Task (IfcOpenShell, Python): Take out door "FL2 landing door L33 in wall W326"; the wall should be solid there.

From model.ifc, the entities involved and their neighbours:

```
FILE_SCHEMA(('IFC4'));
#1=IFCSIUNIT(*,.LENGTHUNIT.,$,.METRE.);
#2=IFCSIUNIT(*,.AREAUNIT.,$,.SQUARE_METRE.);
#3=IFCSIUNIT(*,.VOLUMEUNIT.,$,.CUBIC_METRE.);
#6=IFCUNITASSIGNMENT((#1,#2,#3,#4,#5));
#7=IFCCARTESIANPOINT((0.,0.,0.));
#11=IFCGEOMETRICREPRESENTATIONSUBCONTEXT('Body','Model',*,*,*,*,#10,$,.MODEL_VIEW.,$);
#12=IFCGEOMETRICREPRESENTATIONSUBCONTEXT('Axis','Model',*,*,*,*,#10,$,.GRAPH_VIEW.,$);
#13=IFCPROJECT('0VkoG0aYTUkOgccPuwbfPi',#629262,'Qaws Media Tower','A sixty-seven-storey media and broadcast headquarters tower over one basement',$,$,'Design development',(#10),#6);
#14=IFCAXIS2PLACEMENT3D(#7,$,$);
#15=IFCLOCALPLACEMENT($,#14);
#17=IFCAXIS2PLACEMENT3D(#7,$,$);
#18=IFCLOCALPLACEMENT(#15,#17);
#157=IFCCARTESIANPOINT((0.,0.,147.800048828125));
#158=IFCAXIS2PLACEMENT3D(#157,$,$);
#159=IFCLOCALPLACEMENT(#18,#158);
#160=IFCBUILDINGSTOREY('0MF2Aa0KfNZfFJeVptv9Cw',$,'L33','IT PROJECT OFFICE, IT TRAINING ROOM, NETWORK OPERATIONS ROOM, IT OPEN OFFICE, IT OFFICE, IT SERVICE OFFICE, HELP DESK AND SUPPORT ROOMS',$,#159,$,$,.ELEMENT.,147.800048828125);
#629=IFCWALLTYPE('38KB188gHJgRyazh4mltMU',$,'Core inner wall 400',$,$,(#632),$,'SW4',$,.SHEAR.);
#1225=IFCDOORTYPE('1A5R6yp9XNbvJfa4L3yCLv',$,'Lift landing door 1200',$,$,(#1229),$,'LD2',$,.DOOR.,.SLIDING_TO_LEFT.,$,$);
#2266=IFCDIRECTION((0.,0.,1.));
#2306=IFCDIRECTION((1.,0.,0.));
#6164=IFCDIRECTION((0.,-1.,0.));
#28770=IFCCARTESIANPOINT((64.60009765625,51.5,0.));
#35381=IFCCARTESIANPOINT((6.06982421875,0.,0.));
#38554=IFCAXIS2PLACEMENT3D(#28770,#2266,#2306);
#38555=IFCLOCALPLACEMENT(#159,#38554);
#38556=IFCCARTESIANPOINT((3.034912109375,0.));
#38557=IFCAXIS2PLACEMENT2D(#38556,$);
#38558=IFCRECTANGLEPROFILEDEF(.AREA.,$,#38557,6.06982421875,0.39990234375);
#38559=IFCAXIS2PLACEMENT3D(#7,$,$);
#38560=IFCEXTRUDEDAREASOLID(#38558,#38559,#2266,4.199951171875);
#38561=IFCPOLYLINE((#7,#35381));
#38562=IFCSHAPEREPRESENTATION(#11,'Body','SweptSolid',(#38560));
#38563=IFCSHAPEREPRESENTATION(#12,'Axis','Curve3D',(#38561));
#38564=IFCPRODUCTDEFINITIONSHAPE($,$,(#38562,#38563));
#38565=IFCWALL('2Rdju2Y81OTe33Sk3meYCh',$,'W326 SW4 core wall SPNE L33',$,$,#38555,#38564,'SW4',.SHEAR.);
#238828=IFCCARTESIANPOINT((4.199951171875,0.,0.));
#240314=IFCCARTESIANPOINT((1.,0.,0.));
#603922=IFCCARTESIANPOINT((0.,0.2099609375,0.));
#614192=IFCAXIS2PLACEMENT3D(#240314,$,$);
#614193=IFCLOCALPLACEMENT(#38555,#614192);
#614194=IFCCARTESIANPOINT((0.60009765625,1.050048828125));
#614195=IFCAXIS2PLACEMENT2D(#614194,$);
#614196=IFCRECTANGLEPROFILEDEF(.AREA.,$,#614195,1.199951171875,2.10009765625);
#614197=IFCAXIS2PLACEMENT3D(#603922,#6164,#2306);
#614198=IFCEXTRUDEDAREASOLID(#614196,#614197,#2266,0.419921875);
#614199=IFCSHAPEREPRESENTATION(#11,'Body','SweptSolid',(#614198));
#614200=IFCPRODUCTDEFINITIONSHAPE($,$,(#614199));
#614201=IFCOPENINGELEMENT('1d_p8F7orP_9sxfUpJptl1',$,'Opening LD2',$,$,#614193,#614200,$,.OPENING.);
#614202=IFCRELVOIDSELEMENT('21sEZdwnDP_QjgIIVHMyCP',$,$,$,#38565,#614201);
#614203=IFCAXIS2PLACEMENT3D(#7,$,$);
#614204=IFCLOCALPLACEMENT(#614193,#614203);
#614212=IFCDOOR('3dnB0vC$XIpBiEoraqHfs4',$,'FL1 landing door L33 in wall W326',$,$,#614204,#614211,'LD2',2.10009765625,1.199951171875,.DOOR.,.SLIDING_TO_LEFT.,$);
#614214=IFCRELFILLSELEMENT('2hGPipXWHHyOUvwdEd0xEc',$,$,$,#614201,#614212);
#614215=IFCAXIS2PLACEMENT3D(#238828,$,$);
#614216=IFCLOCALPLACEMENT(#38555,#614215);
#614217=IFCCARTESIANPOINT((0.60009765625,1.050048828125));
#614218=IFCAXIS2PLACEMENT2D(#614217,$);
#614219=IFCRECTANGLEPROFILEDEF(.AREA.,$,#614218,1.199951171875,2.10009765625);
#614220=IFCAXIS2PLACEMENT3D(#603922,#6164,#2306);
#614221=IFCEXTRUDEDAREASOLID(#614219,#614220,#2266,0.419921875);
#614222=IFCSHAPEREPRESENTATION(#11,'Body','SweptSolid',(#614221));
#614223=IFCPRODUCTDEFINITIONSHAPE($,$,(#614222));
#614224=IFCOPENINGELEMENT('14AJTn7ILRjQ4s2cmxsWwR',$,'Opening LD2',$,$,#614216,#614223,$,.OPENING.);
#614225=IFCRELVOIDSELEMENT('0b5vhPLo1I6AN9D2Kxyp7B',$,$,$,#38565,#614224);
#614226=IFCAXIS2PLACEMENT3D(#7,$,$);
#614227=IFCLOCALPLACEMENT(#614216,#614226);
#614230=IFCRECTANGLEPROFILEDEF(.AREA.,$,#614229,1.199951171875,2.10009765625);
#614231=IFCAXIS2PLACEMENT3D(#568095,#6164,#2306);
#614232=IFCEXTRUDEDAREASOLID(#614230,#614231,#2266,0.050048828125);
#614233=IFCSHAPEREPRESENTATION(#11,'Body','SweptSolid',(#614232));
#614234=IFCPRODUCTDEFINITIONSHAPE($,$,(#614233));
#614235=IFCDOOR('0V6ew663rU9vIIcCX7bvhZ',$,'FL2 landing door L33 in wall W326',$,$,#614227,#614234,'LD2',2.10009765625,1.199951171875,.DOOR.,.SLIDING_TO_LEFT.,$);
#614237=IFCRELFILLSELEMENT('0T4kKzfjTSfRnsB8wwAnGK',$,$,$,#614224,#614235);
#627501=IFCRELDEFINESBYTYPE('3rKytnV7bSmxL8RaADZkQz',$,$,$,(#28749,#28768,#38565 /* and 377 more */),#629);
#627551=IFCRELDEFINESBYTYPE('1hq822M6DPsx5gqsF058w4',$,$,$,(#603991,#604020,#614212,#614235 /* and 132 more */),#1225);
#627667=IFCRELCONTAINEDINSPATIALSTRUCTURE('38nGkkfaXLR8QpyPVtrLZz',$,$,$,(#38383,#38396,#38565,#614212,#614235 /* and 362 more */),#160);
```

```python
import ifcopenshell
import ifcopenshell.api.feature
import ifcopenshell.api.root
import ifcopenshell.geom
import ifcopenshell.util.shape

model = ifcopenshell.open("model.ifc")
settings = ifcopenshell.geom.settings()


def volume(element):
    """Net volume in cubic metres, openings subtracted."""
    shape = ifcopenshell.geom.create_shape(settings, element)
    return ifcopenshell.util.shape.get_volume(shape.geometry)


door = model.by_id(614235)
opening = door.FillsVoids[0].RelatingOpeningElement
wall = opening.VoidsElements[0].RelatingBuildingElement
before = volume(wall)

ifcopenshell.api.root.remove_product(model, product=door)
ifcopenshell.api.feature.remove_feature(model, feature=opening)

after = volume(wall)

print(f"wall volume {before:.3f} -> {after:.3f} m3")

model.write("model-out.ifc")
```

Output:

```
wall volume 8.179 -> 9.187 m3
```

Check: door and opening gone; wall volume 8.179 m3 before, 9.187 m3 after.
